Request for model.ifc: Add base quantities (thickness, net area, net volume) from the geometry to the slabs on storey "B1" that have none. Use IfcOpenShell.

First a look at what the model holds.

```python
import ifcopenshell
import ifcopenshell.util.element
import ifcopenshell.util.unit

model = ifcopenshell.open("model.ifc")
print(model.schema)
for unit_type in ("LENGTHUNIT", "AREAUNIT", "VOLUMEUNIT"):
    print(unit_type, ifcopenshell.util.unit.calculate_unit_scale(model, unit_type))
storey = next(s for s in model.by_type("IfcBuildingStorey") if s.Name == "B1")
slabs = [e for e in ifcopenshell.util.element.get_decomposition(storey) if e.is_a("IfcSlab")]
for e in sorted(slabs, key=lambda e: e.id()):
    print(e.id(), e.is_a(), e.Name, list(ifcopenshell.util.element.get_psets(e, qtos_only=True)), sep=" | ")
```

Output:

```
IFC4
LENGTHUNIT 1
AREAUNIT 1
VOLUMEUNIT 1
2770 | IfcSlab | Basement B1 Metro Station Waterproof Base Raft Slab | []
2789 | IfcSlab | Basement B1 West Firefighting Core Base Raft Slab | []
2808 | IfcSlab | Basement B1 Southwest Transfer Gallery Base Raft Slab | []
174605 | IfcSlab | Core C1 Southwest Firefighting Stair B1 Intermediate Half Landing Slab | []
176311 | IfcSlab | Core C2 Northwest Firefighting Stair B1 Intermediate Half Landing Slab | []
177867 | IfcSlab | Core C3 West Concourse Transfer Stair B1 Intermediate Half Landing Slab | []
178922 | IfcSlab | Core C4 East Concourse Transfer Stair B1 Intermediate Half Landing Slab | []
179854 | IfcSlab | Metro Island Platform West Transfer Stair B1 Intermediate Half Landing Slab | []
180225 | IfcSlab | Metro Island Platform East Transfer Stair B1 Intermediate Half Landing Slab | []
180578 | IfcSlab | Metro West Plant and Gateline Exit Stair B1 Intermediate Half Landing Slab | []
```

```python
import ifcopenshell
import ifcopenshell.api.pset
import ifcopenshell.geom
import ifcopenshell.util.element
import ifcopenshell.util.shape
import ifcopenshell.util.unit

model = ifcopenshell.open("model.ifc")
unit_scale = ifcopenshell.util.unit.calculate_unit_scale(model)
area_scale = ifcopenshell.util.unit.calculate_unit_scale(model, "AREAUNIT")
volume_scale = ifcopenshell.util.unit.calculate_unit_scale(model, "VOLUMEUNIT")
settings = ifcopenshell.geom.settings()

storey = next(s for s in model.by_type("IfcBuildingStorey") if s.Name == "B1")
slabs = [e for e in ifcopenshell.util.element.get_decomposition(storey) if e.is_a("IfcSlab")]

for e in sorted(slabs, key=lambda e: e.id()):
    if ifcopenshell.util.element.get_psets(e, qtos_only=True, should_inherit=False):
        continue
    # Geometry comes back in metres, in the element's own axes.
    shape = ifcopenshell.geom.create_shape(settings, e)
    values = {
        "Width": ifcopenshell.util.shape.get_z(shape.geometry) / unit_scale,
        "NetArea": ifcopenshell.util.shape.get_footprint_area(shape.geometry) / area_scale,
        "NetVolume": ifcopenshell.util.shape.get_volume(shape.geometry) / volume_scale,
    }
    qto = ifcopenshell.api.pset.add_qto(model, product=e, name="Qto_SlabBaseQuantities")
    ifcopenshell.api.pset.edit_qto(model, qto=qto, properties=values)
    print(e.id(), {k: round(v, 3) for k, v in values.items()})

model.write("model-out.ifc")
```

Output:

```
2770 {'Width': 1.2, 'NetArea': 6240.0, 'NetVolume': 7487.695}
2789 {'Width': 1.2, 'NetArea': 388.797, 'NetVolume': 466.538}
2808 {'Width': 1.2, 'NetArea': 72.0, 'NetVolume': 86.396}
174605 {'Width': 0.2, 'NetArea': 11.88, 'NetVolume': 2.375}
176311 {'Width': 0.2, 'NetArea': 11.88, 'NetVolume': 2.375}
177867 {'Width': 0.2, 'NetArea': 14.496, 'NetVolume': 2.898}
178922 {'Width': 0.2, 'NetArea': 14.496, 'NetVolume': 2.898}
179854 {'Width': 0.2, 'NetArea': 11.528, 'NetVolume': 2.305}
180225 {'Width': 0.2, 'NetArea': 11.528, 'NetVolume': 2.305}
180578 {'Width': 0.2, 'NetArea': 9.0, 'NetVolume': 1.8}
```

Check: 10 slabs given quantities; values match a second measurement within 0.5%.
